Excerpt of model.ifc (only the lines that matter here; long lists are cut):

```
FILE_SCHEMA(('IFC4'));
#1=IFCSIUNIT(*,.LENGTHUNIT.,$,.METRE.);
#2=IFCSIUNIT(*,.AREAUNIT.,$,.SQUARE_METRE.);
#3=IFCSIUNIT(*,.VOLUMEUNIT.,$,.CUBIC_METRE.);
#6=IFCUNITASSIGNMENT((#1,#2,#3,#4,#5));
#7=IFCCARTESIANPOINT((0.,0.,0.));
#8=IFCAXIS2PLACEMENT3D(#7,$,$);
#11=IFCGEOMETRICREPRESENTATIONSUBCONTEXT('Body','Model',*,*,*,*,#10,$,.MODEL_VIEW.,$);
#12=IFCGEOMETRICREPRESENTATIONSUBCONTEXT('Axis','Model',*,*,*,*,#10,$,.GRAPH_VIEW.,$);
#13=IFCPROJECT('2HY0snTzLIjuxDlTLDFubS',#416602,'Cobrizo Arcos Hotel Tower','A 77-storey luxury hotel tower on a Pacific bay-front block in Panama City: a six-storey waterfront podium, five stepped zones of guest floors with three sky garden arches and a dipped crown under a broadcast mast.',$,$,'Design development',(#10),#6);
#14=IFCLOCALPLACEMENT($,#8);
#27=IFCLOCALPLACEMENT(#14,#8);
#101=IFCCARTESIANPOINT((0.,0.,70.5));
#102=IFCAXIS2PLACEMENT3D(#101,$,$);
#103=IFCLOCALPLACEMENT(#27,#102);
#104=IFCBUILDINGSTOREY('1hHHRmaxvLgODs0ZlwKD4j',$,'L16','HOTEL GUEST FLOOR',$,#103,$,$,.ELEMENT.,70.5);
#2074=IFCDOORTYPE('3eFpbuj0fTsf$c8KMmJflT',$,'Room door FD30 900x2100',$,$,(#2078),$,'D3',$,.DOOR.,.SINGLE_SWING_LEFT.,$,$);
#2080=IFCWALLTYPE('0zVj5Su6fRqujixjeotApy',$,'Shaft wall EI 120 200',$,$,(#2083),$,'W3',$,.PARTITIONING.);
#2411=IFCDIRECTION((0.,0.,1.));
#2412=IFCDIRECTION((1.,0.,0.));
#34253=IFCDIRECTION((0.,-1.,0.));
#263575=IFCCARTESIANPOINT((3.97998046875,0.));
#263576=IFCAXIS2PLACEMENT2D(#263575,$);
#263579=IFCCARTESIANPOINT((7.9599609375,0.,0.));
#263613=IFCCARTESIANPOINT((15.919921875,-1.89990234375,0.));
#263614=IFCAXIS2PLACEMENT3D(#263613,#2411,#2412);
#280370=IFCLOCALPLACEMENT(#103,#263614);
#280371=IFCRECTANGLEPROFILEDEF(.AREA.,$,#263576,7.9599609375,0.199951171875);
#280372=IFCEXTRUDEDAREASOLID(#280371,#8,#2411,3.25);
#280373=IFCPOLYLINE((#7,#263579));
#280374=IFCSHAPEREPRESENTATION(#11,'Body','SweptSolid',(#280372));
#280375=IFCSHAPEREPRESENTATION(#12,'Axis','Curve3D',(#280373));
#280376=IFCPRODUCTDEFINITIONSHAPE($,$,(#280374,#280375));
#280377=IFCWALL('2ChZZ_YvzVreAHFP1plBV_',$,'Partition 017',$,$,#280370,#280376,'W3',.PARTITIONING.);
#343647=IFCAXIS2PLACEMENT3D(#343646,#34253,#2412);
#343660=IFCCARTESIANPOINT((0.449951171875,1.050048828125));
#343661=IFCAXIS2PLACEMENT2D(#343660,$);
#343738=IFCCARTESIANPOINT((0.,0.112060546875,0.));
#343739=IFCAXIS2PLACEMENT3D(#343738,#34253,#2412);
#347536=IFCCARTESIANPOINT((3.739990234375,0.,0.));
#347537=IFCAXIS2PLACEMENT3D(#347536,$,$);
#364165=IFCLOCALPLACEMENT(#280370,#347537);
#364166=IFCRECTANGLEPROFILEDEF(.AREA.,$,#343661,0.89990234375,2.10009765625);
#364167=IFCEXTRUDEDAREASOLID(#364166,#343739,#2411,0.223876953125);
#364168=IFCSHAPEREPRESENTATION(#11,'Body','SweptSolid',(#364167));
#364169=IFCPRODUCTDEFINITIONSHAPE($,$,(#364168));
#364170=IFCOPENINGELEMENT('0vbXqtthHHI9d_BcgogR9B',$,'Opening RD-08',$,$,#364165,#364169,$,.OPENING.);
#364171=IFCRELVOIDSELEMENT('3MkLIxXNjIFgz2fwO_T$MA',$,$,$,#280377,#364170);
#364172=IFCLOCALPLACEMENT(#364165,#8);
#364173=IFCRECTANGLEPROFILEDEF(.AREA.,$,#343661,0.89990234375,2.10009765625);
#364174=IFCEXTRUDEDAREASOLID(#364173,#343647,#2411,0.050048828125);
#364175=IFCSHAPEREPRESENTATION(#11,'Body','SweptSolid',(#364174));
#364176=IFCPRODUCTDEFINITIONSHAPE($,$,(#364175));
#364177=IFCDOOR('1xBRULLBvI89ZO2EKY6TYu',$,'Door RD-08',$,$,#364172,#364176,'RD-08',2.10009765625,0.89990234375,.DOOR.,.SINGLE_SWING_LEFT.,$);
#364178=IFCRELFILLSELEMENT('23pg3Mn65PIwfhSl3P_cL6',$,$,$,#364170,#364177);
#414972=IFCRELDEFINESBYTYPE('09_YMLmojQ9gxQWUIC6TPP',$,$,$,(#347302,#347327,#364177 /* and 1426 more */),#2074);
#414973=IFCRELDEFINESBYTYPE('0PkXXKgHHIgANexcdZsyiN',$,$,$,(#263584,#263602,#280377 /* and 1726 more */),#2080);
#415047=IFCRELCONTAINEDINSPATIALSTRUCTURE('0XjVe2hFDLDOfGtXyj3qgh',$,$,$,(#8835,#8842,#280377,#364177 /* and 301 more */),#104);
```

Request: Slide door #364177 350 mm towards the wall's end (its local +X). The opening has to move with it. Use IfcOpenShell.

```python
import ifcopenshell
import ifcopenshell.api.geometry
import ifcopenshell.util.placement

model = ifcopenshell.open("model.ifc")

door = model.by_id(364177)
opening = door.FillsVoids[0].RelatingOpeningElement
wall = opening.VoidsElements[0].RelatingBuildingElement

wall_matrix = ifcopenshell.util.placement.get_local_placement(wall.ObjectPlacement)
shift = wall_matrix[:3, 0] * 0.35
before = ifcopenshell.util.placement.get_local_placement(door.ObjectPlacement)[:3, 3].copy()

# The door is placed relative to its opening, so it follows when the opening moves.
matrix = ifcopenshell.util.placement.get_local_placement(opening.ObjectPlacement)
matrix[:3, 3] += shift
ifcopenshell.api.geometry.edit_object_placement(
    model, product=opening, matrix=matrix, is_si=False, should_transform_children=True
)

after = ifcopenshell.util.placement.get_local_placement(door.ObjectPlacement)[:3, 3]
print("door moved by", (after - before).round(3) + 0.0)

model.write("model_v2.ifc")
```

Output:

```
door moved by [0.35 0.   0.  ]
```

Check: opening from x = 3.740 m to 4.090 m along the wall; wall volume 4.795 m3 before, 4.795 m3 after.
